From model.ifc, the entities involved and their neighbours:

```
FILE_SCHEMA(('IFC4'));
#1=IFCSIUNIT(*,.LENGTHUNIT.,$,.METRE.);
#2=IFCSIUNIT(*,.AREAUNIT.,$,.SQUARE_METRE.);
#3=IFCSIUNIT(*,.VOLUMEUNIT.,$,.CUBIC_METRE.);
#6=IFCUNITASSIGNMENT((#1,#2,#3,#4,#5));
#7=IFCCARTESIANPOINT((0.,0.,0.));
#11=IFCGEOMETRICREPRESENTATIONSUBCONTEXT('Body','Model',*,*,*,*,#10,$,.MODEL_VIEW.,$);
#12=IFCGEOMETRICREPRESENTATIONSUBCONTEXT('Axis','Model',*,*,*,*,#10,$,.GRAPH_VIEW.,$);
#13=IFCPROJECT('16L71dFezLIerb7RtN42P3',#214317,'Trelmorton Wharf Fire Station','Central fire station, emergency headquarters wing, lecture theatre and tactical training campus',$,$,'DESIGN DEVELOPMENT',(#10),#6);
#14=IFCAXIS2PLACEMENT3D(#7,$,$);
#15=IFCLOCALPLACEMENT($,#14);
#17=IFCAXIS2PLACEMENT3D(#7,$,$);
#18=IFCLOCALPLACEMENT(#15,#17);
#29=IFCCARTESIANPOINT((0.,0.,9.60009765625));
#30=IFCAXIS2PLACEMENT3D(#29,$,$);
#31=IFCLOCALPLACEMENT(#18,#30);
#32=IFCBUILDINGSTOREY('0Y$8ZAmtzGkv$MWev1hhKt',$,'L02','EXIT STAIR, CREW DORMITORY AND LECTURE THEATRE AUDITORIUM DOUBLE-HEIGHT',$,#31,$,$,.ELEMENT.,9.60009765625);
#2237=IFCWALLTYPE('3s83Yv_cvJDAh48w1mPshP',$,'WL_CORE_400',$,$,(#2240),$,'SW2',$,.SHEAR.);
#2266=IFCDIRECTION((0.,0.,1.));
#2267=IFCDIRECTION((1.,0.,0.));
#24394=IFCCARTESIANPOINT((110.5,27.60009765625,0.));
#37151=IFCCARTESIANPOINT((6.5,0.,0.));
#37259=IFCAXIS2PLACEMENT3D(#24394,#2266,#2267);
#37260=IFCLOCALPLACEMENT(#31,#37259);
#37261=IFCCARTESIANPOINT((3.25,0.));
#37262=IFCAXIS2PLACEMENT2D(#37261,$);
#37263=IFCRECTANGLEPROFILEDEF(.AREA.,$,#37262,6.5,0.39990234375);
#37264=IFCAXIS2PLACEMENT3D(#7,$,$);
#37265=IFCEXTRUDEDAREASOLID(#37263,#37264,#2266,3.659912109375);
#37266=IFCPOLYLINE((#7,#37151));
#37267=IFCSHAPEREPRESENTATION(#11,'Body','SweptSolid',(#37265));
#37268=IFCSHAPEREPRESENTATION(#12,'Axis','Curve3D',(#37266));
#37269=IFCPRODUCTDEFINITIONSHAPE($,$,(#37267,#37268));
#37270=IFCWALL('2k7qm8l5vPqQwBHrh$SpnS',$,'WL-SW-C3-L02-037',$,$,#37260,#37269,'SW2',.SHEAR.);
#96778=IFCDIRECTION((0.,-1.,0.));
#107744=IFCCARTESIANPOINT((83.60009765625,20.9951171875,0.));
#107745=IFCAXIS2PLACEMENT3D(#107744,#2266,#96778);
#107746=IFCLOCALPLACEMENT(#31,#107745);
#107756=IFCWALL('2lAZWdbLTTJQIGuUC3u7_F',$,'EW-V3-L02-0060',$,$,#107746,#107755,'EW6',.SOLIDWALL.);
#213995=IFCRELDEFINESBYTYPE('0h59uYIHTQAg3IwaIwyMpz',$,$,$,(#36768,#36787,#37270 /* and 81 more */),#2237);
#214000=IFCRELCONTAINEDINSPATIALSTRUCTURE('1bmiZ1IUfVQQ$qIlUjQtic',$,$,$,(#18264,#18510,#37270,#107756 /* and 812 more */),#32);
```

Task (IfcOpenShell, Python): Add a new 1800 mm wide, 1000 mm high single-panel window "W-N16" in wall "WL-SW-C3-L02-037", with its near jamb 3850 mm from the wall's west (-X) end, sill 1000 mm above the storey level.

```python
import numpy as np
import ifcopenshell
import ifcopenshell.api.feature
import ifcopenshell.api.geometry
import ifcopenshell.api.root
import ifcopenshell.api.spatial
import ifcopenshell.geom
import ifcopenshell.util.element
import ifcopenshell.util.placement
import ifcopenshell.util.representation
import ifcopenshell.util.shape
import ifcopenshell.util.unit

model = ifcopenshell.open("model.ifc")
unit_scale = ifcopenshell.util.unit.calculate_unit_scale(model)
settings = ifcopenshell.geom.settings()


def volume(element):
    """Net volume in cubic metres, openings subtracted."""
    shape = ifcopenshell.geom.create_shape(settings, element)
    return ifcopenshell.util.shape.get_volume(shape.geometry)


wall = model.by_guid("2k7qm8l5vPqQwBHrh$SpnS")
storey = ifcopenshell.util.element.get_container(wall, ifc_class="IfcBuildingStorey")
context = ifcopenshell.util.representation.get_context(model, "Model", "Body", "MODEL_VIEW")
before = volume(wall)

width, height, from_end, sill = 1.8, 1, 3.85, 1  # metres

# The wall runs along its own X axis, and the end named is its -X end.
wall_shape = ifcopenshell.geom.create_shape(settings, wall)
x, y, z = ifcopenshell.util.shape.get_vertices(wall_shape.geometry).T
start = x.min() + from_end
face, thickness = float(y.min()), float(y.max() - y.min())
wall_matrix = ifcopenshell.util.placement.get_local_placement(wall.ObjectPlacement)
level = ifcopenshell.util.placement.get_local_placement(storey.ObjectPlacement)[2, 3]


def in_wall(x, y):
    """Placement at x, y metres in the wall's axes, at sill height."""
    matrix = wall_matrix.copy()
    matrix[:, 3] = wall_matrix @ np.array([x / unit_scale, y / unit_scale, 0.0, 1.0])
    matrix[2, 3] = level + sill / unit_scale
    return matrix


# Opening: a box that overshoots both wall faces by 50 mm.
opening = ifcopenshell.api.root.create_entity(model, ifc_class="IfcOpeningElement", predefined_type="OPENING")
box = ifcopenshell.api.geometry.add_wall_representation(
    model, context=context, length=width, height=height, thickness=thickness + 0.1
)
ifcopenshell.api.geometry.assign_representation(model, product=opening, representation=box)
ifcopenshell.api.geometry.edit_object_placement(model, product=opening, matrix=in_wall(start, face - 0.05), is_si=False)
ifcopenshell.api.feature.add_feature(model, feature=opening, element=wall)

window = ifcopenshell.api.root.create_entity(model, ifc_class="IfcWindow", name="W-N16", predefined_type="WINDOW")
window.OverallWidth, window.OverallHeight = width / unit_scale, height / unit_scale
window.PartitioningType = "SINGLE_PANEL"
body = ifcopenshell.api.geometry.add_window_representation(
    model,
    context=context,
    overall_width=window.OverallWidth,
    overall_height=window.OverallHeight,
    partition_type="SINGLE_PANEL",
)
ifcopenshell.api.geometry.assign_representation(model, product=window, representation=body)
ifcopenshell.api.spatial.assign_container(model, products=[window], relating_structure=storey)
ifcopenshell.api.feature.add_filling(model, opening=opening, element=window)

# Centre the window in the wall's thickness.
ifcopenshell.api.geometry.edit_object_placement(model, product=window, matrix=in_wall(start, face), is_si=False)
window_shape = ifcopenshell.geom.create_shape(settings, window)
depth = ifcopenshell.util.shape.get_vertices(window_shape.geometry)[:, 1]
offset = face + thickness / 2 - (depth.min() + depth.max()) / 2
ifcopenshell.api.geometry.edit_object_placement(model, product=window, matrix=in_wall(start, offset), is_si=False)

after = volume(wall)

print(f"wall volume {before:.3f} -> {after:.3f} m3")

model.write("model-out.ifc")
```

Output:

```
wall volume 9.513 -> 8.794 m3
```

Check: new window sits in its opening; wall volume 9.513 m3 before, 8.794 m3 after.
